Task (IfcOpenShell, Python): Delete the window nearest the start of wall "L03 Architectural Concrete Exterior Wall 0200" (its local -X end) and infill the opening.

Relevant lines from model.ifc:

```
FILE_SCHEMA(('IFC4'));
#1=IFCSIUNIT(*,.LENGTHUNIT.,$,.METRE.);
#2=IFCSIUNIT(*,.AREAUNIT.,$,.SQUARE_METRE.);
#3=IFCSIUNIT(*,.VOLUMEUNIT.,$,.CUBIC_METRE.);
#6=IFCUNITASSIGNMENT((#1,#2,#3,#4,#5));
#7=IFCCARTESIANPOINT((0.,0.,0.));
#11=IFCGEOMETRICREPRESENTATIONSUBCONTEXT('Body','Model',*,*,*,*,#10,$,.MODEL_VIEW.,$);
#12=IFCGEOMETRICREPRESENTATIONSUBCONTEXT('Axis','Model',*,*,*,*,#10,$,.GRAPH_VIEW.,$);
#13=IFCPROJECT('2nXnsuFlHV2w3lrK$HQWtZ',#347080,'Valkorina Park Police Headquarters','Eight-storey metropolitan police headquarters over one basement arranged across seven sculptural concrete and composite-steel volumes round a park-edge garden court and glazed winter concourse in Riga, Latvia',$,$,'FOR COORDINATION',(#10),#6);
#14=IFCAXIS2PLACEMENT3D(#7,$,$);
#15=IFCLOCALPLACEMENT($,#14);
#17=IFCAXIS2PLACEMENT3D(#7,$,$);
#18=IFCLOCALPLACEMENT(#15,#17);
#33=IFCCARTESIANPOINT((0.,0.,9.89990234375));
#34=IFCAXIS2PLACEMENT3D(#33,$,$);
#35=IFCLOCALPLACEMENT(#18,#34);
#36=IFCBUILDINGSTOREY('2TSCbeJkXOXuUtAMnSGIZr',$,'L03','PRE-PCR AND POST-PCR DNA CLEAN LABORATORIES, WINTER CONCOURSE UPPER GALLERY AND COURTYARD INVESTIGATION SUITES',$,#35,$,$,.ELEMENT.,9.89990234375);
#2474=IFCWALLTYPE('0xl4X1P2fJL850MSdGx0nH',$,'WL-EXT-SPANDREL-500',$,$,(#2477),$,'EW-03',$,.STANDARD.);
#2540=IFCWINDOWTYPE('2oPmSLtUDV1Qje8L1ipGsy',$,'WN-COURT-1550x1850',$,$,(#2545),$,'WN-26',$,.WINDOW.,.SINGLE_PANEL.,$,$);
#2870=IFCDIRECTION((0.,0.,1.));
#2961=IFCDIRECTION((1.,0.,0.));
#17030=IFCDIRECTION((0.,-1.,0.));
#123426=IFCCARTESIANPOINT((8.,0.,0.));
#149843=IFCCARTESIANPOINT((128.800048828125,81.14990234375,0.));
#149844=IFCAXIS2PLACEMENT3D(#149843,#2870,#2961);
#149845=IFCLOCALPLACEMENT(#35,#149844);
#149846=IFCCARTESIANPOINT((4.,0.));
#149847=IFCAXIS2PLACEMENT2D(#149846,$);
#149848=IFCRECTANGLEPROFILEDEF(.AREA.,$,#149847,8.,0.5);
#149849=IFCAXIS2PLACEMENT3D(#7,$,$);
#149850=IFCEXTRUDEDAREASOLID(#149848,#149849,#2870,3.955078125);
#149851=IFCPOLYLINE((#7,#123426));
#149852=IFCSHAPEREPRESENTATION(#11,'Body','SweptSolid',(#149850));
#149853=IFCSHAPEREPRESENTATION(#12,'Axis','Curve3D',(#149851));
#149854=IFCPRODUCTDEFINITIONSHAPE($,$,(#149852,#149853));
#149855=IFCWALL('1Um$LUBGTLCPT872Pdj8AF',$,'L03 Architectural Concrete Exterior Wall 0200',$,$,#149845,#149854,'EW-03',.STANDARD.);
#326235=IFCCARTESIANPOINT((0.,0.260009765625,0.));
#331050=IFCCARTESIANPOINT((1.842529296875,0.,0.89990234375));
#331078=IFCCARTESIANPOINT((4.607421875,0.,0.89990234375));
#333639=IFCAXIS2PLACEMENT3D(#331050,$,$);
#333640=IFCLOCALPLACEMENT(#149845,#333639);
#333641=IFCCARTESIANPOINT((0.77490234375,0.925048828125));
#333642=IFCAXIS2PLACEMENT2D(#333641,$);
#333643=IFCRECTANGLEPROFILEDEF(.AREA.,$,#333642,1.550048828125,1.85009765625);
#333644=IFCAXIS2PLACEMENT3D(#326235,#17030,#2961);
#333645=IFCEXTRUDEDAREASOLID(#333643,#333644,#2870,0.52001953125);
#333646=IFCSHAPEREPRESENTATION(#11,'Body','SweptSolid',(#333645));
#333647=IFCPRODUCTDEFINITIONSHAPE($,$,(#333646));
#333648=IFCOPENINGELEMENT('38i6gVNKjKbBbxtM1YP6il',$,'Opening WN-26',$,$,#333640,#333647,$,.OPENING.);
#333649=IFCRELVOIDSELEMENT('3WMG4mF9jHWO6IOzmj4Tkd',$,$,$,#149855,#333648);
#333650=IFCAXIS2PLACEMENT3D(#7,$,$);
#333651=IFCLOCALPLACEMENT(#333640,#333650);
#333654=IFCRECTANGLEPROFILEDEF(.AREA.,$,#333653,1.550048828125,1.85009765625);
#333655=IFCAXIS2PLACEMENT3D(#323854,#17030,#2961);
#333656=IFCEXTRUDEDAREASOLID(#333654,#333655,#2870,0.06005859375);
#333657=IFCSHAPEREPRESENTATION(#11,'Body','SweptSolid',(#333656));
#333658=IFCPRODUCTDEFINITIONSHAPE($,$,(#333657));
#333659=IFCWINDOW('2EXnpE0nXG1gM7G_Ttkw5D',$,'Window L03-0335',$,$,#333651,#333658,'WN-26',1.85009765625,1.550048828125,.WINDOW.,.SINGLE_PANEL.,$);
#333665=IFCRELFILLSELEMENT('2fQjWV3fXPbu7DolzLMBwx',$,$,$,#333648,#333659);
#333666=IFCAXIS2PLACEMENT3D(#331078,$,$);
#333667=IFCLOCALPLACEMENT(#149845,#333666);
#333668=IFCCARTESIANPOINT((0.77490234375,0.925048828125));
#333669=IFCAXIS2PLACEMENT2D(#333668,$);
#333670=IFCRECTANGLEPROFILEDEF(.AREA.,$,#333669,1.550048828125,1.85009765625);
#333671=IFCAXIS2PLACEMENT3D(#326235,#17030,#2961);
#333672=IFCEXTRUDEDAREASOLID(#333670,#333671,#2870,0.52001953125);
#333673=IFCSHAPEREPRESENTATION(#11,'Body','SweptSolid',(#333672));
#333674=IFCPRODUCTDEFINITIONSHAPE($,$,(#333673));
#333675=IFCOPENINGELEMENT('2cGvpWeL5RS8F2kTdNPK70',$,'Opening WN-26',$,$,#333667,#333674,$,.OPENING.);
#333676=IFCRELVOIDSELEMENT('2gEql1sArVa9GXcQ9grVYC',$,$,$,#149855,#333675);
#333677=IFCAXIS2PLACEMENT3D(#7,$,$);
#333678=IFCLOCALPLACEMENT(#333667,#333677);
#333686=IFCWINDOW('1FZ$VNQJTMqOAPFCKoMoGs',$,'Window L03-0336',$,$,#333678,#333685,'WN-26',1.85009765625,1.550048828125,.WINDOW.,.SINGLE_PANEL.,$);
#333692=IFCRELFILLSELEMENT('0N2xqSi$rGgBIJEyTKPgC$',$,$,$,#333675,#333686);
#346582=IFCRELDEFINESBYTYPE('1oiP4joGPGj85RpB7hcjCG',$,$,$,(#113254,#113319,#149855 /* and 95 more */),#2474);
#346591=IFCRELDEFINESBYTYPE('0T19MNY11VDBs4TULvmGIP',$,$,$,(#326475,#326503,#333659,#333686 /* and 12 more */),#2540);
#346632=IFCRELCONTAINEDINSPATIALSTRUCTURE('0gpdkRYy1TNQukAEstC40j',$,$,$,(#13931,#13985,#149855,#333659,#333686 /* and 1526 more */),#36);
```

```python
import ifcopenshell
import ifcopenshell.api.feature
import ifcopenshell.api.root
import ifcopenshell.geom
import ifcopenshell.util.shape

model = ifcopenshell.open("model.ifc")
settings = ifcopenshell.geom.settings()


def volume(element):
    """Net volume in cubic metres, openings subtracted."""
    shape = ifcopenshell.geom.create_shape(settings, element)
    return ifcopenshell.util.shape.get_volume(shape.geometry)


window = model.by_guid("2EXnpE0nXG1gM7G_Ttkw5D")
opening = window.FillsVoids[0].RelatingOpeningElement
wall = opening.VoidsElements[0].RelatingBuildingElement
before = volume(wall)

ifcopenshell.api.root.remove_product(model, product=window)
ifcopenshell.api.feature.remove_feature(model, feature=opening)

after = volume(wall)

print(f"wall volume {before:.3f} -> {after:.3f} m3")

model.write("model_v2.ifc")
```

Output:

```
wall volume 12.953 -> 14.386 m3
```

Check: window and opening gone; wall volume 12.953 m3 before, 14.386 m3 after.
